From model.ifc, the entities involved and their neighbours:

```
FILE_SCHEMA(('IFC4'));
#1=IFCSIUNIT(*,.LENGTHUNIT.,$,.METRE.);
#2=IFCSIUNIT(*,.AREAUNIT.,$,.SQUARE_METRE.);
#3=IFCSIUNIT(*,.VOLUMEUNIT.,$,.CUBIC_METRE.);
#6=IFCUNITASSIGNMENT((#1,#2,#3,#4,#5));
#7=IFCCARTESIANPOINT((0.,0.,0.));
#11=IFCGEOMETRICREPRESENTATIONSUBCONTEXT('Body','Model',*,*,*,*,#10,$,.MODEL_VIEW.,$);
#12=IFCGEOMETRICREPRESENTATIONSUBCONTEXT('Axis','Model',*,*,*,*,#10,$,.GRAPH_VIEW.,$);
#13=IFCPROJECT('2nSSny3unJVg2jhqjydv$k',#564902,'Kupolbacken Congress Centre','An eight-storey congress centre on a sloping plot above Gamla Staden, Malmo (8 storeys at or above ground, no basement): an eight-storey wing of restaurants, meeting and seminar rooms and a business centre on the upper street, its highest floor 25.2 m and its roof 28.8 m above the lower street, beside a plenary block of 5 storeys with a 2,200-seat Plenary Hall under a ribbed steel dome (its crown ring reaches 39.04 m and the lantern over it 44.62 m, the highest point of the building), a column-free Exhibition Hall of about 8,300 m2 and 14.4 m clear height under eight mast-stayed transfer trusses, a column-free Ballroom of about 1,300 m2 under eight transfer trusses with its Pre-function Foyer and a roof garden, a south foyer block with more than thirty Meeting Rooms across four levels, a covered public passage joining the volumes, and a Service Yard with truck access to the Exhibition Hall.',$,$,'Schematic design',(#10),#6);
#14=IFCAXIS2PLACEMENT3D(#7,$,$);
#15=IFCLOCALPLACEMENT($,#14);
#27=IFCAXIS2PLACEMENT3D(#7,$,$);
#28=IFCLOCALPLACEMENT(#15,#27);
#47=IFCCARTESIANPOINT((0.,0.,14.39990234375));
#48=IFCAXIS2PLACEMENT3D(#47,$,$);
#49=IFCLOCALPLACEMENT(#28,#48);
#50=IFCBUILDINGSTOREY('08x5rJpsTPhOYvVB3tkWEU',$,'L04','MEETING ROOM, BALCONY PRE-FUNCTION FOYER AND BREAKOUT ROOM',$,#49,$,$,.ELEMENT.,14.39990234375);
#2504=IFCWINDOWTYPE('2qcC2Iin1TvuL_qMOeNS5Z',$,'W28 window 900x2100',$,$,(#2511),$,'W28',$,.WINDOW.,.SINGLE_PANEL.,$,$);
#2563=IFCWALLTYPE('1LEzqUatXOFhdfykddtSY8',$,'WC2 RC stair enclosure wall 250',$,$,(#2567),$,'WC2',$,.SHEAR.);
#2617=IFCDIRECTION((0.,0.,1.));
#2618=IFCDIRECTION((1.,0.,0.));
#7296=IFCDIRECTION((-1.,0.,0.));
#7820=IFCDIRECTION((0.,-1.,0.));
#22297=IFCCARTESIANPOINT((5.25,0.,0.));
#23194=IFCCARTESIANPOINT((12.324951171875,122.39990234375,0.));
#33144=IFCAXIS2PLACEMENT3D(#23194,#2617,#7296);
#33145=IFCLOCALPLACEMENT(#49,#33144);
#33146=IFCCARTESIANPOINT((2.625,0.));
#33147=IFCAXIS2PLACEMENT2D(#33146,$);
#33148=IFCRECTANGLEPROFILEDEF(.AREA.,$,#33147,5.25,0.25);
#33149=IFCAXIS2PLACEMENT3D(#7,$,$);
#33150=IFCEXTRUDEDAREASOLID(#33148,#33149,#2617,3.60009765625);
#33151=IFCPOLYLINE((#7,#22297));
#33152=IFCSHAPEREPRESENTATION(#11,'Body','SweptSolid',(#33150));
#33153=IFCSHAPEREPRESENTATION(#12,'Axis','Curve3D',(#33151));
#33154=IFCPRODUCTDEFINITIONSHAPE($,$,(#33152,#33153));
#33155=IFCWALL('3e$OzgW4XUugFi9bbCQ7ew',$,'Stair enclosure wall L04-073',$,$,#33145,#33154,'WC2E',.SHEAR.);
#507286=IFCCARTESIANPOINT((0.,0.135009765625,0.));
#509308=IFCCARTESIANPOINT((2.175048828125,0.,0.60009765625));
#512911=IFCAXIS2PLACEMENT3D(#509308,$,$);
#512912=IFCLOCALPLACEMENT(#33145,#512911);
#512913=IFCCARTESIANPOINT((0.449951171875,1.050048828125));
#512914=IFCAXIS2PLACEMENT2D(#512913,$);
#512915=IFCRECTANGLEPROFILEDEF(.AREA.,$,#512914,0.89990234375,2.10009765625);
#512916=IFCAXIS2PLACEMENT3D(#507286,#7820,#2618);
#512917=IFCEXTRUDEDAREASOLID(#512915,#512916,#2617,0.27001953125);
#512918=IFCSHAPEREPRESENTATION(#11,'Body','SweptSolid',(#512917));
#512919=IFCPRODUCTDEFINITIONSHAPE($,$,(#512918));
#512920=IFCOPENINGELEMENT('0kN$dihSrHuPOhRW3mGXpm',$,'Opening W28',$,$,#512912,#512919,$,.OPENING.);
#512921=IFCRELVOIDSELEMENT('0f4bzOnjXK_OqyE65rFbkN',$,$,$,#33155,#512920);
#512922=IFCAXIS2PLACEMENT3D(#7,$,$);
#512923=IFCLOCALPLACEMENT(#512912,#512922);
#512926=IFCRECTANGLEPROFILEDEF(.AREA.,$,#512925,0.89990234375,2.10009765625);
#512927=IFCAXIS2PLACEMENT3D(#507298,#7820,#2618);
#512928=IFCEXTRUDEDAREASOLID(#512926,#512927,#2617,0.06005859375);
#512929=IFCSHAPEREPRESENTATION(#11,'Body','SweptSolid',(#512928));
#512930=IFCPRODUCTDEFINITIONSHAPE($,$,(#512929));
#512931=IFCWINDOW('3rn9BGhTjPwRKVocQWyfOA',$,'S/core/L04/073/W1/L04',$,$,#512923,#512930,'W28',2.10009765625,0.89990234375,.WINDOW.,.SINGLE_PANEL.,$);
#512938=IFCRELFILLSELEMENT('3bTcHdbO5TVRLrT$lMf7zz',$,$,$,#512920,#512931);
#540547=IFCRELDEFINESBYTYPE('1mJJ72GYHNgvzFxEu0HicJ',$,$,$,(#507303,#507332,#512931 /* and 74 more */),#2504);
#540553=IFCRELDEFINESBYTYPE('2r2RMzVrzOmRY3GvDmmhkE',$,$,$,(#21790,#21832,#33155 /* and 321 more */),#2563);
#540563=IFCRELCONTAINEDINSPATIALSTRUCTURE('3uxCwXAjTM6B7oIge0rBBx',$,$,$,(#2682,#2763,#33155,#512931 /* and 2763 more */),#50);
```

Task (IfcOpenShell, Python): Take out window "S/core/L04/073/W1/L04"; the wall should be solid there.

```python
import ifcopenshell
import ifcopenshell.api.feature
import ifcopenshell.api.root
import ifcopenshell.geom
import ifcopenshell.util.shape

model = ifcopenshell.open("model.ifc")
settings = ifcopenshell.geom.settings()


def volume(element):
    """Net volume in cubic metres, openings subtracted."""
    shape = ifcopenshell.geom.create_shape(settings, element)
    return ifcopenshell.util.shape.get_volume(shape.geometry)


window = model.by_guid("3rn9BGhTjPwRKVocQWyfOA")
opening = window.FillsVoids[0].RelatingOpeningElement
wall = opening.VoidsElements[0].RelatingBuildingElement
before = volume(wall)

ifcopenshell.api.root.remove_product(model, product=window)
ifcopenshell.api.feature.remove_feature(model, feature=opening)

after = volume(wall)

print(f"wall volume {before:.3f} -> {after:.3f} m3")

model.write("model_edited.ifc")
```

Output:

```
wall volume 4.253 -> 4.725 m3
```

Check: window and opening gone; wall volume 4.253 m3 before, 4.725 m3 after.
